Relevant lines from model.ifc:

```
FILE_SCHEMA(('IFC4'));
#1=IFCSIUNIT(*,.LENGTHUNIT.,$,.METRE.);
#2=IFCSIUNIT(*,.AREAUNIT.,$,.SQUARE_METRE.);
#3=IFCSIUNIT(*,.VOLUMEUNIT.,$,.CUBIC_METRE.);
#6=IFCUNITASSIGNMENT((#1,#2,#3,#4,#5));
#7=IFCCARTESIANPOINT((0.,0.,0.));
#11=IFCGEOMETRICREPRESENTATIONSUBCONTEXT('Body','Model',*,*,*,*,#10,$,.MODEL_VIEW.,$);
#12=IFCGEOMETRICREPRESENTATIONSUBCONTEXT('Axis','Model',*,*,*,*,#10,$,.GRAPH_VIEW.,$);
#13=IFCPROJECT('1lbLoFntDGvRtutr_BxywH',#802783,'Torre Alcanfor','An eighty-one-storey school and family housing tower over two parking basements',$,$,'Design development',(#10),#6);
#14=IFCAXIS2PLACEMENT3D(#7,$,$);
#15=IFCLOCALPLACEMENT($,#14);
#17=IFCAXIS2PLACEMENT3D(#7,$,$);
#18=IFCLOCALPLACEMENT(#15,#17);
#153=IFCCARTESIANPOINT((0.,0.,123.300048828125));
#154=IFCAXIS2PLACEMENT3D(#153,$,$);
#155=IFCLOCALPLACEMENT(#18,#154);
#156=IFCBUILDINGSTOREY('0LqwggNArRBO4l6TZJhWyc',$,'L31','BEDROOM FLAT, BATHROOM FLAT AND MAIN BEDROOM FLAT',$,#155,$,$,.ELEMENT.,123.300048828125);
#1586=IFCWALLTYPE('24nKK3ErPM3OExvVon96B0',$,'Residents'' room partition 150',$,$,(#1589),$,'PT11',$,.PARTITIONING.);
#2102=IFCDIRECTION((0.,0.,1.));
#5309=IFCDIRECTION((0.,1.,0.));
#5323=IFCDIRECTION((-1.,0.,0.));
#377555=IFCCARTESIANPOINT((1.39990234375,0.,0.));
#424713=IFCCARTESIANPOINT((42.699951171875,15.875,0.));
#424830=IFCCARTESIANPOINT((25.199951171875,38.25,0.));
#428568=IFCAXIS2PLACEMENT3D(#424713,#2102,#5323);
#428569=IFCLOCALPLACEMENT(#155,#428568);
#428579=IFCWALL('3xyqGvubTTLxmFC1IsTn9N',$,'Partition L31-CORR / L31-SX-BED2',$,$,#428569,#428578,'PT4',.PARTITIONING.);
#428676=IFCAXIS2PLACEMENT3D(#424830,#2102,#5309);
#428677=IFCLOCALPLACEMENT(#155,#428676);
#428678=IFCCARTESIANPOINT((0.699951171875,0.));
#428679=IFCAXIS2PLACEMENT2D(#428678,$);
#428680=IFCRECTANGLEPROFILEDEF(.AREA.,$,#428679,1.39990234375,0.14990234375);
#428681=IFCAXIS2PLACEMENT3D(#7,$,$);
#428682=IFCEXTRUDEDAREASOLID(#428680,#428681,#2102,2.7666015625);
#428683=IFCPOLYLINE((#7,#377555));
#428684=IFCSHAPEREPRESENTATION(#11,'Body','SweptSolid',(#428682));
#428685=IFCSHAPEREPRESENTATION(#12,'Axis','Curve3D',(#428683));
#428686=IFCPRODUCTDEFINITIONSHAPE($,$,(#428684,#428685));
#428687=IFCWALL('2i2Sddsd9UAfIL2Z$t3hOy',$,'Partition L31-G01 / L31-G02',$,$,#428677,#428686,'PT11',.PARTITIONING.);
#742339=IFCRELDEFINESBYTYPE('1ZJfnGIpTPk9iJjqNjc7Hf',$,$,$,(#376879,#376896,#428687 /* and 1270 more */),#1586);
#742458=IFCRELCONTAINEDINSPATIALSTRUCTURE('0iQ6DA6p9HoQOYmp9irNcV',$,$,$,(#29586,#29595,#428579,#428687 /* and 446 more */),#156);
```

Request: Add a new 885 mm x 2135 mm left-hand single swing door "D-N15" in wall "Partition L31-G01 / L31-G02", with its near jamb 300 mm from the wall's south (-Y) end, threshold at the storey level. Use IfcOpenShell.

```python
import numpy as np
import ifcopenshell
import ifcopenshell.api.feature
import ifcopenshell.api.geometry
import ifcopenshell.api.root
import ifcopenshell.api.spatial
import ifcopenshell.geom
import ifcopenshell.util.element
import ifcopenshell.util.placement
import ifcopenshell.util.representation
import ifcopenshell.util.shape
import ifcopenshell.util.unit

model = ifcopenshell.open("model.ifc")
unit_scale = ifcopenshell.util.unit.calculate_unit_scale(model)
settings = ifcopenshell.geom.settings()


def volume(element):
    """Net volume in cubic metres, openings subtracted."""
    shape = ifcopenshell.geom.create_shape(settings, element)
    return ifcopenshell.util.shape.get_volume(shape.geometry)


wall = model.by_id(428687)
storey = ifcopenshell.util.element.get_container(wall, ifc_class="IfcBuildingStorey")
context = ifcopenshell.util.representation.get_context(model, "Model", "Body", "MODEL_VIEW")
before = volume(wall)

width, height, from_end, sill = 0.885, 2.135, 0.3, 0.0  # metres

# The wall runs along its own X axis, and the end named is its -X end.
wall_shape = ifcopenshell.geom.create_shape(settings, wall)
x, y, z = ifcopenshell.util.shape.get_vertices(wall_shape.geometry).T
start = x.min() + from_end
face, thickness = float(y.min()), float(y.max() - y.min())
wall_matrix = ifcopenshell.util.placement.get_local_placement(wall.ObjectPlacement)
level = ifcopenshell.util.placement.get_local_placement(storey.ObjectPlacement)[2, 3]


def in_wall(x, y):
    """Placement at x, y metres in the wall's axes, at sill height."""
    matrix = wall_matrix.copy()
    matrix[:, 3] = wall_matrix @ np.array([x / unit_scale, y / unit_scale, 0.0, 1.0])
    matrix[2, 3] = level + sill / unit_scale
    return matrix


# Opening: a box that overshoots both wall faces by 50 mm.
opening = ifcopenshell.api.root.create_entity(model, ifc_class="IfcOpeningElement", predefined_type="OPENING")
box = ifcopenshell.api.geometry.add_wall_representation(
    model, context=context, length=width, height=height, thickness=thickness + 0.1
)
ifcopenshell.api.geometry.assign_representation(model, product=opening, representation=box)
ifcopenshell.api.geometry.edit_object_placement(model, product=opening, matrix=in_wall(start, face - 0.05), is_si=False)
ifcopenshell.api.feature.add_feature(model, feature=opening, element=wall)

door = ifcopenshell.api.root.create_entity(model, ifc_class="IfcDoor", name="D-N15", predefined_type="DOOR")
door.OverallWidth, door.OverallHeight = width / unit_scale, height / unit_scale
door.OperationType = "SINGLE_SWING_LEFT"
body = ifcopenshell.api.geometry.add_door_representation(
    model,
    context=context,
    overall_width=door.OverallWidth,
    overall_height=door.OverallHeight,
    operation_type="SINGLE_SWING_LEFT",
    lining_properties={"LiningDepth": thickness / unit_scale, "ThresholdDepth": thickness / unit_scale},
)
ifcopenshell.api.geometry.assign_representation(model, product=door, representation=body)
ifcopenshell.api.spatial.assign_container(model, products=[door], relating_structure=storey)
ifcopenshell.api.feature.add_filling(model, opening=opening, element=door)

# The lining spans the wall, so the door starts at the wall face.
ifcopenshell.api.geometry.edit_object_placement(model, product=door, matrix=in_wall(start, face), is_si=False)

after = volume(wall)

print(f"wall volume {before:.3f} -> {after:.3f} m3")

model.write("model_v2.ifc")
```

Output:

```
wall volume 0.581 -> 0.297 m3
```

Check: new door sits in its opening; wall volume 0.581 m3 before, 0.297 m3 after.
